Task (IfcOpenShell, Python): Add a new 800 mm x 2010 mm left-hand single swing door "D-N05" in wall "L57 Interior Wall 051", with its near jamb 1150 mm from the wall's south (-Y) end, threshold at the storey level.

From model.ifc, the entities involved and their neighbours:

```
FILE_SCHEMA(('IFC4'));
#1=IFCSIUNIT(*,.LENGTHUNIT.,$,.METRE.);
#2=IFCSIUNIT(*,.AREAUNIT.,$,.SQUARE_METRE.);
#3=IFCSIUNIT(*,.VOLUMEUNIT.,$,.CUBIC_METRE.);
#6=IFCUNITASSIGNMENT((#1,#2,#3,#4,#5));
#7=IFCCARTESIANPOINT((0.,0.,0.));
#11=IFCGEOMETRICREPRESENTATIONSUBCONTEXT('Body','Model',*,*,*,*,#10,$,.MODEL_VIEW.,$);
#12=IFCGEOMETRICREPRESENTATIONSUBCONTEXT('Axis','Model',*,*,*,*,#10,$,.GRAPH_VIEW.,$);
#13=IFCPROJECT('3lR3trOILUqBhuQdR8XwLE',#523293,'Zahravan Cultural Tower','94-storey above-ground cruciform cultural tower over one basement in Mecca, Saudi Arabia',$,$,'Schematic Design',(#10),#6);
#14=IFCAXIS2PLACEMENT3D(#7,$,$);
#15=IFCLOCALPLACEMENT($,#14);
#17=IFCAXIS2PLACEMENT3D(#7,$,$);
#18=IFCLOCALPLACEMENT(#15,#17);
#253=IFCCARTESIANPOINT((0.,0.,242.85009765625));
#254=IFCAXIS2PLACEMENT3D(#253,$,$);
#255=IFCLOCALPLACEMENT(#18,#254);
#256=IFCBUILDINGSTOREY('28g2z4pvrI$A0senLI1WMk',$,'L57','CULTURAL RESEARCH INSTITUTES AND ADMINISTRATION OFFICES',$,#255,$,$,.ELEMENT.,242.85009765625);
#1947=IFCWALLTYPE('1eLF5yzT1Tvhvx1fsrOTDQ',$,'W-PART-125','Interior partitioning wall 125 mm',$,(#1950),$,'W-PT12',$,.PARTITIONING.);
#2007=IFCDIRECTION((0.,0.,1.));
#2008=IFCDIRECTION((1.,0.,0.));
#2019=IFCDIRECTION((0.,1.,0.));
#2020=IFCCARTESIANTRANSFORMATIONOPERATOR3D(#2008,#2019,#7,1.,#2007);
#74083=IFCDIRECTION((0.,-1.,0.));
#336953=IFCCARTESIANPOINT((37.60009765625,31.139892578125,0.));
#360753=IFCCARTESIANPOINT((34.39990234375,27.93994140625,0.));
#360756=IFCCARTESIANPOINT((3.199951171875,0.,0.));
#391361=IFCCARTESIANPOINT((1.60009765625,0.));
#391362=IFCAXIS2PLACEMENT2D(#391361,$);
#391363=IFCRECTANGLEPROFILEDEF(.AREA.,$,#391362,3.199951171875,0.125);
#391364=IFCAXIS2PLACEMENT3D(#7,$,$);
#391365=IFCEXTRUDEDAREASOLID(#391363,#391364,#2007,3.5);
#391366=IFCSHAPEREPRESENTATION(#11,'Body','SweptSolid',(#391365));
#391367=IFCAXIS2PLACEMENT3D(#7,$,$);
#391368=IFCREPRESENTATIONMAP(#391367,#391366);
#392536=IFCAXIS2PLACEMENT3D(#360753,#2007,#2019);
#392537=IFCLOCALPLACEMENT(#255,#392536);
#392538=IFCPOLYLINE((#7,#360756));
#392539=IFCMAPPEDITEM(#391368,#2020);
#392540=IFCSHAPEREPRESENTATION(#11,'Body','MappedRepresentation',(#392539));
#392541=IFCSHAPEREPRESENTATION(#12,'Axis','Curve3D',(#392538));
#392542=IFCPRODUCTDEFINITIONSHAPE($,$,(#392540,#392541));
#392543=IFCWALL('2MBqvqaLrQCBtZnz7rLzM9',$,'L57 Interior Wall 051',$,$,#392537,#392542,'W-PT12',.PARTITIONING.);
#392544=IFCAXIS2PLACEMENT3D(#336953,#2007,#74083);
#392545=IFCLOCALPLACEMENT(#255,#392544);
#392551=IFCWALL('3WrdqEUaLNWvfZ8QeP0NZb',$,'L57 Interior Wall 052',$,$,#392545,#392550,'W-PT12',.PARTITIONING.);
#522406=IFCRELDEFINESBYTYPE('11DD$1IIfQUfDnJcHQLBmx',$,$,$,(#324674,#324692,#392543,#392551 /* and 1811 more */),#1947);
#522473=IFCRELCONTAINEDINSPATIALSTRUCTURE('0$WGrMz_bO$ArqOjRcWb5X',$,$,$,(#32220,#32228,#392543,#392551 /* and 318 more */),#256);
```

```python
import numpy as np
import ifcopenshell
import ifcopenshell.api.feature
import ifcopenshell.api.geometry
import ifcopenshell.api.root
import ifcopenshell.api.spatial
import ifcopenshell.geom
import ifcopenshell.util.element
import ifcopenshell.util.placement
import ifcopenshell.util.representation
import ifcopenshell.util.shape
import ifcopenshell.util.unit

model = ifcopenshell.open("model.ifc")
unit_scale = ifcopenshell.util.unit.calculate_unit_scale(model)
settings = ifcopenshell.geom.settings()


def volume(element):
    """Net volume in cubic metres, openings subtracted."""
    shape = ifcopenshell.geom.create_shape(settings, element)
    return ifcopenshell.util.shape.get_volume(shape.geometry)


wall = model.by_id(392543)
storey = ifcopenshell.util.element.get_container(wall, ifc_class="IfcBuildingStorey")
context = ifcopenshell.util.representation.get_context(model, "Model", "Body", "MODEL_VIEW")
before = volume(wall)

width, height, from_end, sill = 0.8, 2.01, 1.15, 0.0  # metres

# The wall runs along its own X axis, and the end named is its -X end.
wall_shape = ifcopenshell.geom.create_shape(settings, wall)
x, y, z = ifcopenshell.util.shape.get_vertices(wall_shape.geometry).T
start = x.min() + from_end
face, thickness = float(y.min()), float(y.max() - y.min())
wall_matrix = ifcopenshell.util.placement.get_local_placement(wall.ObjectPlacement)
level = ifcopenshell.util.placement.get_local_placement(storey.ObjectPlacement)[2, 3]


def in_wall(x, y):
    """Placement at x, y metres in the wall's axes, at sill height."""
    matrix = wall_matrix.copy()
    matrix[:, 3] = wall_matrix @ np.array([x / unit_scale, y / unit_scale, 0.0, 1.0])
    matrix[2, 3] = level + sill / unit_scale
    return matrix


# Opening: a box that overshoots both wall faces by 50 mm.
opening = ifcopenshell.api.root.create_entity(model, ifc_class="IfcOpeningElement", predefined_type="OPENING")
box = ifcopenshell.api.geometry.add_wall_representation(
    model, context=context, length=width, height=height, thickness=thickness + 0.1
)
ifcopenshell.api.geometry.assign_representation(model, product=opening, representation=box)
ifcopenshell.api.geometry.edit_object_placement(model, product=opening, matrix=in_wall(start, face - 0.05), is_si=False)
ifcopenshell.api.feature.add_feature(model, feature=opening, element=wall)

door = ifcopenshell.api.root.create_entity(model, ifc_class="IfcDoor", name="D-N05", predefined_type="DOOR")
door.OverallWidth, door.OverallHeight = width / unit_scale, height / unit_scale
door.OperationType = "SINGLE_SWING_LEFT"
body = ifcopenshell.api.geometry.add_door_representation(
    model,
    context=context,
    overall_width=door.OverallWidth,
    overall_height=door.OverallHeight,
    operation_type="SINGLE_SWING_LEFT",
    lining_properties={"LiningDepth": thickness / unit_scale, "ThresholdDepth": thickness / unit_scale},
)
ifcopenshell.api.geometry.assign_representation(model, product=door, representation=body)
ifcopenshell.api.spatial.assign_container(model, products=[door], relating_structure=storey)
ifcopenshell.api.feature.add_filling(model, opening=opening, element=door)

# The lining spans the wall, so the door starts at the wall face.
ifcopenshell.api.geometry.edit_object_placement(model, product=door, matrix=in_wall(start, face), is_si=False)

after = volume(wall)

print(f"wall volume {before:.3f} -> {after:.3f} m3")

model.write("model_updated.ifc")
```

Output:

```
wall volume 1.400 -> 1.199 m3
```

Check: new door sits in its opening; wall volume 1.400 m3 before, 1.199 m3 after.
